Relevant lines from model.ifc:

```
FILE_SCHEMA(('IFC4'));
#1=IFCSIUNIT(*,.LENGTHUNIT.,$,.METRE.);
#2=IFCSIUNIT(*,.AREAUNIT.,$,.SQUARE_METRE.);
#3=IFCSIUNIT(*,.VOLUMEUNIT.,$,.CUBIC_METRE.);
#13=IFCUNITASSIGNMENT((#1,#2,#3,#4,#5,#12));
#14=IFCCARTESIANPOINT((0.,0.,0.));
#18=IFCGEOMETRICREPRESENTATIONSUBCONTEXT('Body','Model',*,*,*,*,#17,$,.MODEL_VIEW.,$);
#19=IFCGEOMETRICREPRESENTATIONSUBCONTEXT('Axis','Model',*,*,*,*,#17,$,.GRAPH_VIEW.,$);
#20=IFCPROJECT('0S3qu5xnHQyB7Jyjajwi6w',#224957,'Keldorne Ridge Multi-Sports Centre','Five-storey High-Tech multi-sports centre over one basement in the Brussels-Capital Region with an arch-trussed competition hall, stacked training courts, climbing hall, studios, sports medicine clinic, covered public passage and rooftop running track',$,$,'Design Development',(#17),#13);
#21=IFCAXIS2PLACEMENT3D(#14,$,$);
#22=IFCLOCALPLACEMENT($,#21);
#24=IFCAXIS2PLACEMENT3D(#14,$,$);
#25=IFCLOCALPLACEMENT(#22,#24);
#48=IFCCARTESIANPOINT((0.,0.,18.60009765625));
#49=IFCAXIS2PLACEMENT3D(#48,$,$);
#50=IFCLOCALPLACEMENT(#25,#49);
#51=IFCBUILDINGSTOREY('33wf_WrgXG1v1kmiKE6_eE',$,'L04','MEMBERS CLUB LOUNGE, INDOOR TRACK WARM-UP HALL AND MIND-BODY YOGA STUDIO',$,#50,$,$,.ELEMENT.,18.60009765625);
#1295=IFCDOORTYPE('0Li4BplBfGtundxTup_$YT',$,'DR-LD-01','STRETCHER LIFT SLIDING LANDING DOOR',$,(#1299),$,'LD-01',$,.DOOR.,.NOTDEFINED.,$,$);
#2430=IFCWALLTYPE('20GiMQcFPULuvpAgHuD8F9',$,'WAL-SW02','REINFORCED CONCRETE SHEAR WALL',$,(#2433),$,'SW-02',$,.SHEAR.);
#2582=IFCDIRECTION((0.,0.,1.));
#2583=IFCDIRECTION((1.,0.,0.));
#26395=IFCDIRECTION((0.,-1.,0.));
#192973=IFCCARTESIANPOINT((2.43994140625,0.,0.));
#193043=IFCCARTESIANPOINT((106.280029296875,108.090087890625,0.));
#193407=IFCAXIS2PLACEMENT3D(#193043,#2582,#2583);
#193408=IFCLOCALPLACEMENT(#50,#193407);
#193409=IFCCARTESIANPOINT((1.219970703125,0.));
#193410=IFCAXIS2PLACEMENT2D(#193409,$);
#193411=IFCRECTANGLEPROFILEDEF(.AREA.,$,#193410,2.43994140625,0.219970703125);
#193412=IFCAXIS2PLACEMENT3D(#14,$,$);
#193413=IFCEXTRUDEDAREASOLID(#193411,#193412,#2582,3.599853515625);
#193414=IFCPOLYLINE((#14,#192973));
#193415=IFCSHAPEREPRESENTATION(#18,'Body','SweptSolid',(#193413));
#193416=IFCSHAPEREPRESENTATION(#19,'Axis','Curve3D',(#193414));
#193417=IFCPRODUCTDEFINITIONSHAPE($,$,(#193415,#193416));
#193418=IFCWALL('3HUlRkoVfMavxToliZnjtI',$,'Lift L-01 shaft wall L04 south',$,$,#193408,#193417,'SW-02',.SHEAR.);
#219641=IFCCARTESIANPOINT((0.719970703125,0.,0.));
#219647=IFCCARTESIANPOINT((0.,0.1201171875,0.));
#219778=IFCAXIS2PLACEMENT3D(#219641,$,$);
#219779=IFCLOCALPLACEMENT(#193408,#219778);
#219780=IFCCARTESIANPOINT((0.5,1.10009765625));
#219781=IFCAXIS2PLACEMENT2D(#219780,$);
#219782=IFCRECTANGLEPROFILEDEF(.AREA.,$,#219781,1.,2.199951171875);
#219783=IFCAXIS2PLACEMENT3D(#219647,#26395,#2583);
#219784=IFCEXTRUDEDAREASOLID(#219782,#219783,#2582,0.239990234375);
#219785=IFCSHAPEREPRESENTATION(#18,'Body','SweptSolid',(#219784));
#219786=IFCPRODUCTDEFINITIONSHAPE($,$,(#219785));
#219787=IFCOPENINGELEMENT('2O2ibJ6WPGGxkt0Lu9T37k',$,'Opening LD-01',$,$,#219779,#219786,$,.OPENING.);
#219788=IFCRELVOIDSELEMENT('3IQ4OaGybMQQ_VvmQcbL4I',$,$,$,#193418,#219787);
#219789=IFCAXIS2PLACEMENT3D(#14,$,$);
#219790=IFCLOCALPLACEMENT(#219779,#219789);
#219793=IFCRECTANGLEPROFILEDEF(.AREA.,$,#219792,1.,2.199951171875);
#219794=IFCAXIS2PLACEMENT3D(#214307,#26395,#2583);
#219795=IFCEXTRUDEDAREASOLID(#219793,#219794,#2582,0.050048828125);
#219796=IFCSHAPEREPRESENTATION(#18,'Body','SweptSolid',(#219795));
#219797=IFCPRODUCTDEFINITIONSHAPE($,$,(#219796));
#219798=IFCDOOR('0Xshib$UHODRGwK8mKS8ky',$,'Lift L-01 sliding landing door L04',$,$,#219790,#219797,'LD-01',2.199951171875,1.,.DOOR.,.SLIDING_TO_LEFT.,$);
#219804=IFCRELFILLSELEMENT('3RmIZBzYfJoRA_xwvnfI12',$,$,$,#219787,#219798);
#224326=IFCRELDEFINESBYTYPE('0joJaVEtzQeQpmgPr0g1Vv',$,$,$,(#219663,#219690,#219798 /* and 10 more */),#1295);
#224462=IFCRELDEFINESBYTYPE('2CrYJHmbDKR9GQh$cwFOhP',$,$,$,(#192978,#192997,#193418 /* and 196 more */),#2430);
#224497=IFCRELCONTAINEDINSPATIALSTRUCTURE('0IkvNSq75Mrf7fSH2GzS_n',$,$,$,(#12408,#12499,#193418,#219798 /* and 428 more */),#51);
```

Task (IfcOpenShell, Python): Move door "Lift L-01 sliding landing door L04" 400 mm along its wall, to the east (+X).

```python
import ifcopenshell
import ifcopenshell.api.geometry
import ifcopenshell.util.placement
import ifcopenshell.util.unit

model = ifcopenshell.open("model.ifc")
unit_scale = ifcopenshell.util.unit.calculate_unit_scale(model)

door = model.by_guid("0Xshib$UHODRGwK8mKS8ky")
opening = door.FillsVoids[0].RelatingOpeningElement
wall = opening.VoidsElements[0].RelatingBuildingElement

wall_matrix = ifcopenshell.util.placement.get_local_placement(wall.ObjectPlacement)
shift = wall_matrix[:3, 0] * 0.4 / unit_scale
before = ifcopenshell.util.placement.get_local_placement(door.ObjectPlacement)[:3, 3].copy()

# The door is placed relative to its opening, so it follows when the opening moves.
matrix = ifcopenshell.util.placement.get_local_placement(opening.ObjectPlacement)
matrix[:3, 3] += shift
ifcopenshell.api.geometry.edit_object_placement(
    model, product=opening, matrix=matrix, is_si=False, should_transform_children=True
)

after = ifcopenshell.util.placement.get_local_placement(door.ObjectPlacement)[:3, 3]
print("door moved by", (after - before).round(3) + 0.0)

model.write("model_edited.ifc")
```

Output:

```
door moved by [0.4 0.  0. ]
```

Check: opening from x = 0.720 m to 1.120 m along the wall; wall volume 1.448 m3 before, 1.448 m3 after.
